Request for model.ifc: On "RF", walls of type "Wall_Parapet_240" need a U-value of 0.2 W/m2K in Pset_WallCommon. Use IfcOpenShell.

First a look at what the model holds.

```python
import ifcopenshell
import ifcopenshell.util.element

model = ifcopenshell.open("model.ifc")
print(model.schema)
storey = next(s for s in model.by_type("IfcBuildingStorey") if s.Name == "RF")
walls = [e for e in ifcopenshell.util.element.get_decomposition(storey) if e.is_a("IfcWall")]
seen = {}
for e in walls:
    element_type = ifcopenshell.util.element.get_type(e)
    key = (element_type.Name if element_type != e and element_type else None, ifcopenshell.util.element.get_pset(e, "Pset_WallCommon", "ThermalTransmittance"))
    seen[key] = seen.get(key, 0) + 1
for (name, value), count in sorted(seen.items(), key=str):
    print(count, "x", name, "|", value)
```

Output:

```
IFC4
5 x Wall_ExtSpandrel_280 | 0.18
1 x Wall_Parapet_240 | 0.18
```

```python
import ifcopenshell
import ifcopenshell.api.pset
import ifcopenshell.util.element

model = ifcopenshell.open("model.ifc")

storey = next(s for s in model.by_type("IfcBuildingStorey") if s.Name == "RF")
walls = [e for e in ifcopenshell.util.element.get_decomposition(storey) if e.is_a("IfcWall")]

count = 0
for e in walls:
    element_type = ifcopenshell.util.element.get_type(e)
    if element_type in (None, e) or element_type.Name != "Wall_Parapet_240":
        continue
    # add_pset returns the element's existing set when there is one.
    pset = ifcopenshell.api.pset.add_pset(model, product=e, name="Pset_WallCommon")
    ifcopenshell.api.pset.edit_pset(model, pset=pset, properties={"ThermalTransmittance": 0.2})
    count += 1

print(count, "walls updated")

model.write("model-out.ifc")
```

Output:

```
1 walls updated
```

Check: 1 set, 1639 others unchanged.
